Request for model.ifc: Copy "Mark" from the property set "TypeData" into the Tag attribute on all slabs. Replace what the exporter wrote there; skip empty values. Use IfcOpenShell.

First a look at what the model holds.

```python
import ifcopenshell
import ifcopenshell.util.element

model = ifcopenshell.open("model.ifc")
print(model.schema)
slabs = model.by_type("IfcSlab")
print(len(slabs), "slabs")
for e in slabs[:8]:
    source = ifcopenshell.util.element.get_pset(e, "TypeData", "Mark")
    target = e.Tag
    print(e.id(), repr(source), repr(target), sep=" | ")
```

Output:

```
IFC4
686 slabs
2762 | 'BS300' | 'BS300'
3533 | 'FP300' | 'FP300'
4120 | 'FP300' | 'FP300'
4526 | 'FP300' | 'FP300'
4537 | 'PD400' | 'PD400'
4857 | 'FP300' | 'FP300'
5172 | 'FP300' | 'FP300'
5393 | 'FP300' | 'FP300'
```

```python
import ifcopenshell
import ifcopenshell.util.element

model = ifcopenshell.open("model.ifc")

count = 0
for e in model.by_type("IfcSlab"):
    value = ifcopenshell.util.element.get_pset(e, "TypeData", "Mark")
    current = e.Tag
    if not value or not value.strip() or current == value:
        continue
    e.Tag = value
    count += 1

print(count, "slabs updated")

model.write("model-out.ifc")
```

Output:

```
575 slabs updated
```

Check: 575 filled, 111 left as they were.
